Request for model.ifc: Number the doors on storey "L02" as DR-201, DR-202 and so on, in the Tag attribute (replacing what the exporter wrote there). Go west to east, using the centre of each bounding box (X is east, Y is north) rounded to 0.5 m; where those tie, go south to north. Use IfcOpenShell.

First a look at what the model holds.

```python
import ifcopenshell
import ifcopenshell.util.element
import ifcopenshell.util.placement

model = ifcopenshell.open("model.ifc")
print(model.schema)
storey = next(s for s in model.by_type("IfcBuildingStorey") if s.Name == "L02")
doors = [e for e in ifcopenshell.util.element.get_decomposition(storey) if e.is_a("IfcDoor")]
for e in sorted(doors, key=lambda e: e.id()):
    origin = ifcopenshell.util.placement.get_local_placement(e.ObjectPlacement)[:3, 3]
    print(e.id(), e.Tag, e.Name, origin.round(2) + 0.0, sep=" | ")
```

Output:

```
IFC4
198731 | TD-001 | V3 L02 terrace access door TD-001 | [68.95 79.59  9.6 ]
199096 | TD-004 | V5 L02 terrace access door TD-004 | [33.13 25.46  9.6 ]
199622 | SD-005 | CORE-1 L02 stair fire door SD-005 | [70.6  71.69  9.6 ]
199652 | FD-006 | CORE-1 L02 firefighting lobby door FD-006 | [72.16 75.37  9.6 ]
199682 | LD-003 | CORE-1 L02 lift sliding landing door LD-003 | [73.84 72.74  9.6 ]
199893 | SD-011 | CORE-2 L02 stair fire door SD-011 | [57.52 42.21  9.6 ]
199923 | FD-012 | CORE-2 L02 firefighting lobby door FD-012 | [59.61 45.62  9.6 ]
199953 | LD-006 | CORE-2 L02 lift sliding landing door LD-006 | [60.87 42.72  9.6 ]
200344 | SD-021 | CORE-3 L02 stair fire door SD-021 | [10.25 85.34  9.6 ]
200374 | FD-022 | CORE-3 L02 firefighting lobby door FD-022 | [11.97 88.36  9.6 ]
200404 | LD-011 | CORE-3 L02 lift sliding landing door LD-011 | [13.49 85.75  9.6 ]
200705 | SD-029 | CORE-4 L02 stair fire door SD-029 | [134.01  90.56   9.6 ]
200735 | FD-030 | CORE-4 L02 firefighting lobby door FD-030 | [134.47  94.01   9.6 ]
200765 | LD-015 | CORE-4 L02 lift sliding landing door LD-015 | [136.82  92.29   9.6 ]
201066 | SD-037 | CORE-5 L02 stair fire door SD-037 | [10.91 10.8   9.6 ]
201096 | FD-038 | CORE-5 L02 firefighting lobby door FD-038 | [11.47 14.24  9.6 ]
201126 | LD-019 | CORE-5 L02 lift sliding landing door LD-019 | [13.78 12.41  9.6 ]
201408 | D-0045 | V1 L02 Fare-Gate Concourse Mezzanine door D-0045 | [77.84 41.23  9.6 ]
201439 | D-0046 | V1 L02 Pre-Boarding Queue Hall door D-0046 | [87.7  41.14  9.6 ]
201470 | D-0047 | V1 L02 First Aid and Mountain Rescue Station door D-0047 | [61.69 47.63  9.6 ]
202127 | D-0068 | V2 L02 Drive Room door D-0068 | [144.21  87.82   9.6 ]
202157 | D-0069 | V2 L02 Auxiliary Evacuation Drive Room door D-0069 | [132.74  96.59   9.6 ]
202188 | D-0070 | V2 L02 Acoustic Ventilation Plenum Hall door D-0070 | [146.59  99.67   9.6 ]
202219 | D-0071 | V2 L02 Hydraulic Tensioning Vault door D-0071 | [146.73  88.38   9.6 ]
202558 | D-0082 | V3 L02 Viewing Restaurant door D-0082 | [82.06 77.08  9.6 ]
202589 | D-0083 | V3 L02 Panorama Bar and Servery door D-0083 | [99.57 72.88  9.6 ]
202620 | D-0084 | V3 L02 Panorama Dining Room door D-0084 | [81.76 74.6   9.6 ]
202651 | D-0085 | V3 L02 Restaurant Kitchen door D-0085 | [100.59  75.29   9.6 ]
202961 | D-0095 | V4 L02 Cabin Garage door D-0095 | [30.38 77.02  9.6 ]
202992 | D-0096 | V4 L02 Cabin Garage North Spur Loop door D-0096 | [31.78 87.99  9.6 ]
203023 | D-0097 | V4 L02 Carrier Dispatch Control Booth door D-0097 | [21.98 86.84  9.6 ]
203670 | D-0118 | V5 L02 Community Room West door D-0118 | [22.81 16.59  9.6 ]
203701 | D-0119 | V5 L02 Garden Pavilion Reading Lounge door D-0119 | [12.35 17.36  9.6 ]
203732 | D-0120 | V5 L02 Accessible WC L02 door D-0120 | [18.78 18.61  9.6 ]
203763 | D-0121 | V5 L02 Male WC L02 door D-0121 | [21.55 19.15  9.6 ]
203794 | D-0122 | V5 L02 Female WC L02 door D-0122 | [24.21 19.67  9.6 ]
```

```python
import ifcopenshell
import ifcopenshell.geom
import ifcopenshell.util.element
import ifcopenshell.util.shape

model = ifcopenshell.open("model.ifc")
settings = ifcopenshell.geom.settings()
settings.set("use-world-coords", True)


def centre(element):
    shape = ifcopenshell.geom.create_shape(settings, element)
    return ifcopenshell.util.shape.get_bbox_centroid(shape.geometry)


storey = next(s for s in model.by_type("IfcBuildingStorey") if s.Name == "L02")
doors = [e for e in ifcopenshell.util.element.get_decomposition(storey) if e.is_a("IfcDoor")]

# Insertion points can sit at a corner or the storey origin, so sort by the geometry (in metres).
centres = {e: centre(e) for e in doors}
doors.sort(key=lambda e: (round(centres[e][0] / 0.5), centres[e][1]))

for i, e in enumerate(doors, start=1):
    number = f"DR-2{i:02d}"
    e.Tag = number
    print(e.id(), number)

model.write("model_rev.ifc")
```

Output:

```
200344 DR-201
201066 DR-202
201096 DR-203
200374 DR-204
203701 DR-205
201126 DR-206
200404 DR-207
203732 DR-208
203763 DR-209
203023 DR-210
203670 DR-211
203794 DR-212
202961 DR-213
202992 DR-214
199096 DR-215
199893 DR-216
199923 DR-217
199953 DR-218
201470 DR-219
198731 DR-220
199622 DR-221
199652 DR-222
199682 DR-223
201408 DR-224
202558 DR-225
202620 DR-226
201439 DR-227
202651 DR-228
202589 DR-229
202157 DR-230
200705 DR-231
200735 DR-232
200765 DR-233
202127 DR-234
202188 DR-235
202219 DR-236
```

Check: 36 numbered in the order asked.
